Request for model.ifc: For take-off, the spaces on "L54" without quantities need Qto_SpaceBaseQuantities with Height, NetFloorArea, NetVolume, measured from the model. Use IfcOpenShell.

First a look at what the model holds.

```python
import ifcopenshell
import ifcopenshell.util.element
import ifcopenshell.util.unit

model = ifcopenshell.open("model.ifc")
print(model.schema)
for unit_type in ("LENGTHUNIT", "AREAUNIT", "VOLUMEUNIT"):
    print(unit_type, ifcopenshell.util.unit.calculate_unit_scale(model, unit_type))
storey = next(s for s in model.by_type("IfcBuildingStorey") if s.Name == "L54")
spaces = [e for e in ifcopenshell.util.element.get_decomposition(storey) if e.is_a("IfcSpace")]
for e in sorted(spaces, key=lambda e: e.id()):
    print(e.id(), e.is_a(), e.Name, list(ifcopenshell.util.element.get_psets(e, qtos_only=True)), sep=" | ")
```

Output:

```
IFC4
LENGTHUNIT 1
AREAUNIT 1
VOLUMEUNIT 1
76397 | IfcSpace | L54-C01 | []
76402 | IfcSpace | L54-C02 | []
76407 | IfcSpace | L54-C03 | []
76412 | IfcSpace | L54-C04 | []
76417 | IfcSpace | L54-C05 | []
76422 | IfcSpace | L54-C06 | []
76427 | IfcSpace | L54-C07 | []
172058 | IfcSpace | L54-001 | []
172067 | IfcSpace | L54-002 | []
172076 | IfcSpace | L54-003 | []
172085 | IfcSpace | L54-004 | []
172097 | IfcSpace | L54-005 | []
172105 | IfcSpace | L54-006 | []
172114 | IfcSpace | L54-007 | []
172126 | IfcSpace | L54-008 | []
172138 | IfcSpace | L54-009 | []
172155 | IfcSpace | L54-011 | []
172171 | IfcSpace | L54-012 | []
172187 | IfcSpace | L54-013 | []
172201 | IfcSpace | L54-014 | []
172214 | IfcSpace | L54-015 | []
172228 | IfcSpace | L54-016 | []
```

```python
import ifcopenshell
import ifcopenshell.api.pset
import ifcopenshell.geom
import ifcopenshell.util.element
import ifcopenshell.util.shape
import ifcopenshell.util.unit

model = ifcopenshell.open("model.ifc")
unit_scale = ifcopenshell.util.unit.calculate_unit_scale(model)
area_scale = ifcopenshell.util.unit.calculate_unit_scale(model, "AREAUNIT")
volume_scale = ifcopenshell.util.unit.calculate_unit_scale(model, "VOLUMEUNIT")
settings = ifcopenshell.geom.settings()

storey = next(s for s in model.by_type("IfcBuildingStorey") if s.Name == "L54")
spaces = [e for e in ifcopenshell.util.element.get_decomposition(storey) if e.is_a("IfcSpace")]

for e in sorted(spaces, key=lambda e: e.id()):
    if ifcopenshell.util.element.get_psets(e, qtos_only=True, should_inherit=False):
        continue
    # Geometry comes back in metres, in the element's own axes.
    shape = ifcopenshell.geom.create_shape(settings, e)
    values = {
        "Height": ifcopenshell.util.shape.get_z(shape.geometry) / unit_scale,
        "NetFloorArea": ifcopenshell.util.shape.get_footprint_area(shape.geometry) / area_scale,
        "NetVolume": ifcopenshell.util.shape.get_volume(shape.geometry) / volume_scale,
    }
    qto = ifcopenshell.api.pset.add_qto(model, product=e, name="Qto_SpaceBaseQuantities")
    ifcopenshell.api.pset.edit_qto(model, qto=qto, properties=values)
    print(e.id(), {k: round(v, 3) for k, v in values.items()})

model.write("model-out.ifc")
```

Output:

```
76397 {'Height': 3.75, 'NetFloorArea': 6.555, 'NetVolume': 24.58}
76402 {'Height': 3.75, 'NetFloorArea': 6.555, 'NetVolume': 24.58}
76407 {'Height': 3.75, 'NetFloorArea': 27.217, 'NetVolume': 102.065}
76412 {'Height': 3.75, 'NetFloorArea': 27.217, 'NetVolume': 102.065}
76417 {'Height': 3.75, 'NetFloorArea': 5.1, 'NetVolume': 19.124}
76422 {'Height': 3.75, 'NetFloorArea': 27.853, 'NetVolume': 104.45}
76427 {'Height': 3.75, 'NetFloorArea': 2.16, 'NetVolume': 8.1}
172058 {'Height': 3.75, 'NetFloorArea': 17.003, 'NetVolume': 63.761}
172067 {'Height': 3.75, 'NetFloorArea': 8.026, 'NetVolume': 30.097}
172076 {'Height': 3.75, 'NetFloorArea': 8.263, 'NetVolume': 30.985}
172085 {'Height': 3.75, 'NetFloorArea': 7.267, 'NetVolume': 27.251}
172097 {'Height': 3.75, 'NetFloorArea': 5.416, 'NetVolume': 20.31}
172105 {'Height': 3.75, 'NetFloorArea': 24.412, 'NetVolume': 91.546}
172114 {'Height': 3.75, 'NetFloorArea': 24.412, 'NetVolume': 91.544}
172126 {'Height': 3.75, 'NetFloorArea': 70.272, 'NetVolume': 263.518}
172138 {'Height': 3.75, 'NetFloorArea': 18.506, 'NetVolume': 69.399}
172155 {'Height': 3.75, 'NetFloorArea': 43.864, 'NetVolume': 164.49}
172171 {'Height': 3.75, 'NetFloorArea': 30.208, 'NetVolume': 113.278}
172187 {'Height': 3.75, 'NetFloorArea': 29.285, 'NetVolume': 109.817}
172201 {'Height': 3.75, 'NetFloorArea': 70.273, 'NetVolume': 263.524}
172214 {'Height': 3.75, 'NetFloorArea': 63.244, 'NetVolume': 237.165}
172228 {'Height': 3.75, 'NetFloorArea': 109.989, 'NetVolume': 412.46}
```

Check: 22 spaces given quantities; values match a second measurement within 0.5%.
